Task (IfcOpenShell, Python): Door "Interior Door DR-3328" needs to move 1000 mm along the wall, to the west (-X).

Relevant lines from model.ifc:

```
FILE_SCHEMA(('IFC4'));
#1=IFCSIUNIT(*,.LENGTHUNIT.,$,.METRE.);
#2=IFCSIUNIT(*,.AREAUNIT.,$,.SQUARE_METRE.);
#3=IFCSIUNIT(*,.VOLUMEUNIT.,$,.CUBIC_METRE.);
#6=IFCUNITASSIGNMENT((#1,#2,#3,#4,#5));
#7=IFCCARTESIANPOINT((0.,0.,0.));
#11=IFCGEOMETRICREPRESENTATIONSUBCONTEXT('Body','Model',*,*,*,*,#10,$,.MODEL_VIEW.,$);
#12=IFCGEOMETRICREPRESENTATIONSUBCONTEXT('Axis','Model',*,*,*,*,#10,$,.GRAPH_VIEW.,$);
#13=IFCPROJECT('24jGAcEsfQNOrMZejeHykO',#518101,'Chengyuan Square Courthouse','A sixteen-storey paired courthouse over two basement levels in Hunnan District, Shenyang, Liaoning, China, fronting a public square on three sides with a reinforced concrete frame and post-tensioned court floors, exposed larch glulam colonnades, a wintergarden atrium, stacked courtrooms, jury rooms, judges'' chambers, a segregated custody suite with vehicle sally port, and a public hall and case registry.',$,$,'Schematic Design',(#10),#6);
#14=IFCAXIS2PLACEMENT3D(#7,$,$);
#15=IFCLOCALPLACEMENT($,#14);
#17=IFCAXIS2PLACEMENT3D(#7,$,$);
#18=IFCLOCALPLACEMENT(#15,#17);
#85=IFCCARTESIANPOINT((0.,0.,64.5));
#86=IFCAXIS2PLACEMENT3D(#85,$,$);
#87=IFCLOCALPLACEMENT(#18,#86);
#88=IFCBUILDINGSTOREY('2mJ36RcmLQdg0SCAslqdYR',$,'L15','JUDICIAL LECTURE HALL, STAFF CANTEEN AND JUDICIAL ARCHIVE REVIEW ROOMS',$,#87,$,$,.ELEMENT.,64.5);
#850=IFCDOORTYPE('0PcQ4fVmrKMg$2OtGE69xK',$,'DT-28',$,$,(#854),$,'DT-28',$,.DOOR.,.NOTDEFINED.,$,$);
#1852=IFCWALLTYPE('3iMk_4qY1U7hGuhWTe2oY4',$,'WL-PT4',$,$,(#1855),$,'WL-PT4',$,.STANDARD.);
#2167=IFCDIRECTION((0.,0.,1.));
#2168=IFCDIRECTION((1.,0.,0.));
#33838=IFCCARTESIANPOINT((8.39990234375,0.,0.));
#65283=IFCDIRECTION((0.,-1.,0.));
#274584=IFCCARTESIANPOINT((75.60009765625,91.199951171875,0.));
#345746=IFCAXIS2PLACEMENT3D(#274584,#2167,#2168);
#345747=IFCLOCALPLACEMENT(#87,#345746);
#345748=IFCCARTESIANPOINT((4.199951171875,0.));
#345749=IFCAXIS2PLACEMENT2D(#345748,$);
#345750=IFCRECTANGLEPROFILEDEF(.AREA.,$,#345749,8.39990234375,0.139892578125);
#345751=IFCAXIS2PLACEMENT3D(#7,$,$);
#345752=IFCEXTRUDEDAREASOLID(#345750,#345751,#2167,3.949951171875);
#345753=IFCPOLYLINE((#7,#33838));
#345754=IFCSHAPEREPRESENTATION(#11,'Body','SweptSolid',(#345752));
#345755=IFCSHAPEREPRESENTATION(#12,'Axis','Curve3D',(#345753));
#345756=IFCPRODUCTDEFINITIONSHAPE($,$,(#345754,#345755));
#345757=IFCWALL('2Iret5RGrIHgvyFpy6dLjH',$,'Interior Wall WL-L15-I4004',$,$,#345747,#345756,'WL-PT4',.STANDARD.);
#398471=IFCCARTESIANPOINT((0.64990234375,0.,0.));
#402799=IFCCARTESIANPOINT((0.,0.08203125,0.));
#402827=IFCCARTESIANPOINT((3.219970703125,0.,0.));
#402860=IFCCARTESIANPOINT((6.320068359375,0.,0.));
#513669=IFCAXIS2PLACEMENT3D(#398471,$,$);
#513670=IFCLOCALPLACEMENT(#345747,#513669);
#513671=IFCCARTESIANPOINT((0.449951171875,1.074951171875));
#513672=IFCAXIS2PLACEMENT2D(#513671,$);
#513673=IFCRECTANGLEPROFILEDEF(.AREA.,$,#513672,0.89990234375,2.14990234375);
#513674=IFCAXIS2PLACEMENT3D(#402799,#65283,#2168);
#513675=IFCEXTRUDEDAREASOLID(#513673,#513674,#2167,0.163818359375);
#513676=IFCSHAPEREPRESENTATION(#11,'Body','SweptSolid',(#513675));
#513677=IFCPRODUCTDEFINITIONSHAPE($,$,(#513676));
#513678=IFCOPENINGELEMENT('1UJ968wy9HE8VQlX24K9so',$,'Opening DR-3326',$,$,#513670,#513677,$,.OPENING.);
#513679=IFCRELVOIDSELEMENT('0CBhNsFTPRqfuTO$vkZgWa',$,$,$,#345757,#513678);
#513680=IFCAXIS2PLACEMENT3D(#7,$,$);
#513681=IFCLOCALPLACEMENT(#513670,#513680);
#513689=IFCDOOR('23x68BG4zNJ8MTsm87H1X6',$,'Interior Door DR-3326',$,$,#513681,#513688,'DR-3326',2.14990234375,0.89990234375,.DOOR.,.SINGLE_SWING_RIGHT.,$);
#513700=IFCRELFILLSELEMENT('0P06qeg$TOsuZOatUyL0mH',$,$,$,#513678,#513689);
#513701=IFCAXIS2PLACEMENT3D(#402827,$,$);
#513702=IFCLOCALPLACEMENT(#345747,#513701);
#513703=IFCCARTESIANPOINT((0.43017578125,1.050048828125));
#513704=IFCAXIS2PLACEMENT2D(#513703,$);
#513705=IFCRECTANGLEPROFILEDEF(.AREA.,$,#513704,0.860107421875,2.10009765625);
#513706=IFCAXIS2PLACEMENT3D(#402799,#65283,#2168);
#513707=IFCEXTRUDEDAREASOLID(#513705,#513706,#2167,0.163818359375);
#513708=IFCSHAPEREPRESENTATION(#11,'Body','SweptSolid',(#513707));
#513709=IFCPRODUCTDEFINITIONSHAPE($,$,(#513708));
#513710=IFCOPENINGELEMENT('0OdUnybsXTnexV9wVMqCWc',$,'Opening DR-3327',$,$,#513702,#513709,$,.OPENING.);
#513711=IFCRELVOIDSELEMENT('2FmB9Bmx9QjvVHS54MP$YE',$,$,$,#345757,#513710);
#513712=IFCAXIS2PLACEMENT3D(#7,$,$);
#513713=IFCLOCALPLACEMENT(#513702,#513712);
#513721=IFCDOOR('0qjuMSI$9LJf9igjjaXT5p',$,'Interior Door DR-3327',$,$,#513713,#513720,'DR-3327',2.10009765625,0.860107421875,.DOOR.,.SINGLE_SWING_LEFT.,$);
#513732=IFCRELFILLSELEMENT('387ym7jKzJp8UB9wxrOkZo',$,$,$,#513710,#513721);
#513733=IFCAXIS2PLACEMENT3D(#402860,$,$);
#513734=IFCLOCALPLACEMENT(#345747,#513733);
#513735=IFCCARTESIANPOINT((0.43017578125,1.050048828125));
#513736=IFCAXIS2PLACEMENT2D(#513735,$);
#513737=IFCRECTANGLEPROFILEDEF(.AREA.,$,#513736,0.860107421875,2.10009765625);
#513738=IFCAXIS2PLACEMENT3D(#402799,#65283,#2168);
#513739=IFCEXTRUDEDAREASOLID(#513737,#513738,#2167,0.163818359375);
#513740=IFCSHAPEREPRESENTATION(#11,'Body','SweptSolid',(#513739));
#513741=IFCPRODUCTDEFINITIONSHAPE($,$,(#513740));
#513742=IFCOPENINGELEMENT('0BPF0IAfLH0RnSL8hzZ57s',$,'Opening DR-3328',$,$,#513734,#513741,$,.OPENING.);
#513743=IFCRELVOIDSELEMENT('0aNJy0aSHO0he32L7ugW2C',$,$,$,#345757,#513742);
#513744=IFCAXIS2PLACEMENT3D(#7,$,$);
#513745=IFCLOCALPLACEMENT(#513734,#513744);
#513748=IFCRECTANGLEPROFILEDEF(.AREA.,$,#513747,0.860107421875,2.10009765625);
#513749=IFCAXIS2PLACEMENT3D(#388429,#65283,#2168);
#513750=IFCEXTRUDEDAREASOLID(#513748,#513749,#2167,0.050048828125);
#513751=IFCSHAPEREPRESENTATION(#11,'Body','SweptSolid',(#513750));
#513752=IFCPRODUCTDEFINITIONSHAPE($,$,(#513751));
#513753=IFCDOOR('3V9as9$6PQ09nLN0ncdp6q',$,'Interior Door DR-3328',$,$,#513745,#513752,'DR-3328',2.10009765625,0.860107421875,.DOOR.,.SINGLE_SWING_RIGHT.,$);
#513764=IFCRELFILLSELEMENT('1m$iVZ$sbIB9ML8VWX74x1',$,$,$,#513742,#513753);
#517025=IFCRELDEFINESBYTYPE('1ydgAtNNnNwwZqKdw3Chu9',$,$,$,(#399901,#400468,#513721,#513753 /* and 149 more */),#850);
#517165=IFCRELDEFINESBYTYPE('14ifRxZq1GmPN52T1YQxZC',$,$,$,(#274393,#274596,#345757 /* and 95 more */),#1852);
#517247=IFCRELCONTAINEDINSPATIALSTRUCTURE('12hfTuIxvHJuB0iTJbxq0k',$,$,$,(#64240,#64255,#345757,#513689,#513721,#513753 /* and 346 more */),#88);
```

```python
import ifcopenshell
import ifcopenshell.api.geometry
import ifcopenshell.util.placement
import ifcopenshell.util.unit

model = ifcopenshell.open("model.ifc")
unit_scale = ifcopenshell.util.unit.calculate_unit_scale(model)

door = model.by_guid("3V9as9$6PQ09nLN0ncdp6q")
opening = door.FillsVoids[0].RelatingOpeningElement
wall = opening.VoidsElements[0].RelatingBuildingElement

wall_matrix = ifcopenshell.util.placement.get_local_placement(wall.ObjectPlacement)
shift = wall_matrix[:3, 0] * -1 / unit_scale
before = ifcopenshell.util.placement.get_local_placement(door.ObjectPlacement)[:3, 3].copy()

# The door is placed relative to its opening, so it follows when the opening moves.
matrix = ifcopenshell.util.placement.get_local_placement(opening.ObjectPlacement)
matrix[:3, 3] += shift
ifcopenshell.api.geometry.edit_object_placement(
    model, product=opening, matrix=matrix, is_si=False, should_transform_children=True
)

after = ifcopenshell.util.placement.get_local_placement(door.ObjectPlacement)[:3, 3]
print("door moved by", (after - before).round(3) + 0.0)

model.write("model_v2.ifc")
```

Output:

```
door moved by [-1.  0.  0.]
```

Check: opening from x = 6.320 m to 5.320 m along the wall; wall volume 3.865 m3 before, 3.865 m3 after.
